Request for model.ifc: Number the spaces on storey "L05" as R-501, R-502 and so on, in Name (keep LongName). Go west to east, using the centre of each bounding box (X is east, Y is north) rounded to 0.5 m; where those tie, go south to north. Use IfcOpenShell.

First a look at what the model holds.

```python
import ifcopenshell
import ifcopenshell.util.element
import ifcopenshell.util.placement

model = ifcopenshell.open("model.ifc")
print(model.schema)
storey = next(s for s in model.by_type("IfcBuildingStorey") if s.Name == "L05")
spaces = [e for e in ifcopenshell.util.element.get_decomposition(storey) if e.is_a("IfcSpace")]
for e in sorted(spaces, key=lambda e: e.id()):
    origin = ifcopenshell.util.placement.get_local_placement(e.ObjectPlacement)[:3, 3]
    print(e.id(), e.Name, e.LongName, origin.round(2) + 0.0, sep=" | ")
```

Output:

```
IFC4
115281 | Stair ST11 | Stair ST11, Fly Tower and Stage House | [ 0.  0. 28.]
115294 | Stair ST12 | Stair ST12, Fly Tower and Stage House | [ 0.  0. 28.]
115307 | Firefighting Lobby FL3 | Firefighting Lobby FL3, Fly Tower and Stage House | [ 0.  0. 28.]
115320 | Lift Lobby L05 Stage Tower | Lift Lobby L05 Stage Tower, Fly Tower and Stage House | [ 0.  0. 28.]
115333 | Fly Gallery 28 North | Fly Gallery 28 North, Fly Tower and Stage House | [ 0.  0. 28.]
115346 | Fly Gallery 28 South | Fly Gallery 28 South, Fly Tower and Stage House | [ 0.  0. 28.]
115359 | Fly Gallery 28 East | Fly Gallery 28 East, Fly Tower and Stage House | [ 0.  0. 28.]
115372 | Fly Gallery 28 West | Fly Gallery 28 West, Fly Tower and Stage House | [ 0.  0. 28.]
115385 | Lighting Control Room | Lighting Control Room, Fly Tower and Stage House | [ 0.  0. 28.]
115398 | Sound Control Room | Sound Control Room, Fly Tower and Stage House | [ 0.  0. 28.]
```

```python
import ifcopenshell
import ifcopenshell.geom
import ifcopenshell.util.element
import ifcopenshell.util.shape

model = ifcopenshell.open("model.ifc")
settings = ifcopenshell.geom.settings()
settings.set("use-world-coords", True)


def centre(element):
    shape = ifcopenshell.geom.create_shape(settings, element)
    return ifcopenshell.util.shape.get_bbox_centroid(shape.geometry)


storey = next(s for s in model.by_type("IfcBuildingStorey") if s.Name == "L05")
spaces = [e for e in ifcopenshell.util.element.get_decomposition(storey) if e.is_a("IfcSpace")]

# Insertion points can sit at a corner or the storey origin, so sort by the geometry (in metres).
centres = {e: centre(e) for e in spaces}
spaces.sort(key=lambda e: (round(centres[e][0] / 0.5), centres[e][1]))

for i, e in enumerate(spaces, start=1):
    number = f"R-5{i:02d}"
    e.Name = number
    print(e.id(), number)

model.write("model_edited.ifc")
```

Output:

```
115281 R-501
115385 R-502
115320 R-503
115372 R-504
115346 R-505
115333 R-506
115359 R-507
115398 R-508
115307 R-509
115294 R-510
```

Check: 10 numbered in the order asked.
